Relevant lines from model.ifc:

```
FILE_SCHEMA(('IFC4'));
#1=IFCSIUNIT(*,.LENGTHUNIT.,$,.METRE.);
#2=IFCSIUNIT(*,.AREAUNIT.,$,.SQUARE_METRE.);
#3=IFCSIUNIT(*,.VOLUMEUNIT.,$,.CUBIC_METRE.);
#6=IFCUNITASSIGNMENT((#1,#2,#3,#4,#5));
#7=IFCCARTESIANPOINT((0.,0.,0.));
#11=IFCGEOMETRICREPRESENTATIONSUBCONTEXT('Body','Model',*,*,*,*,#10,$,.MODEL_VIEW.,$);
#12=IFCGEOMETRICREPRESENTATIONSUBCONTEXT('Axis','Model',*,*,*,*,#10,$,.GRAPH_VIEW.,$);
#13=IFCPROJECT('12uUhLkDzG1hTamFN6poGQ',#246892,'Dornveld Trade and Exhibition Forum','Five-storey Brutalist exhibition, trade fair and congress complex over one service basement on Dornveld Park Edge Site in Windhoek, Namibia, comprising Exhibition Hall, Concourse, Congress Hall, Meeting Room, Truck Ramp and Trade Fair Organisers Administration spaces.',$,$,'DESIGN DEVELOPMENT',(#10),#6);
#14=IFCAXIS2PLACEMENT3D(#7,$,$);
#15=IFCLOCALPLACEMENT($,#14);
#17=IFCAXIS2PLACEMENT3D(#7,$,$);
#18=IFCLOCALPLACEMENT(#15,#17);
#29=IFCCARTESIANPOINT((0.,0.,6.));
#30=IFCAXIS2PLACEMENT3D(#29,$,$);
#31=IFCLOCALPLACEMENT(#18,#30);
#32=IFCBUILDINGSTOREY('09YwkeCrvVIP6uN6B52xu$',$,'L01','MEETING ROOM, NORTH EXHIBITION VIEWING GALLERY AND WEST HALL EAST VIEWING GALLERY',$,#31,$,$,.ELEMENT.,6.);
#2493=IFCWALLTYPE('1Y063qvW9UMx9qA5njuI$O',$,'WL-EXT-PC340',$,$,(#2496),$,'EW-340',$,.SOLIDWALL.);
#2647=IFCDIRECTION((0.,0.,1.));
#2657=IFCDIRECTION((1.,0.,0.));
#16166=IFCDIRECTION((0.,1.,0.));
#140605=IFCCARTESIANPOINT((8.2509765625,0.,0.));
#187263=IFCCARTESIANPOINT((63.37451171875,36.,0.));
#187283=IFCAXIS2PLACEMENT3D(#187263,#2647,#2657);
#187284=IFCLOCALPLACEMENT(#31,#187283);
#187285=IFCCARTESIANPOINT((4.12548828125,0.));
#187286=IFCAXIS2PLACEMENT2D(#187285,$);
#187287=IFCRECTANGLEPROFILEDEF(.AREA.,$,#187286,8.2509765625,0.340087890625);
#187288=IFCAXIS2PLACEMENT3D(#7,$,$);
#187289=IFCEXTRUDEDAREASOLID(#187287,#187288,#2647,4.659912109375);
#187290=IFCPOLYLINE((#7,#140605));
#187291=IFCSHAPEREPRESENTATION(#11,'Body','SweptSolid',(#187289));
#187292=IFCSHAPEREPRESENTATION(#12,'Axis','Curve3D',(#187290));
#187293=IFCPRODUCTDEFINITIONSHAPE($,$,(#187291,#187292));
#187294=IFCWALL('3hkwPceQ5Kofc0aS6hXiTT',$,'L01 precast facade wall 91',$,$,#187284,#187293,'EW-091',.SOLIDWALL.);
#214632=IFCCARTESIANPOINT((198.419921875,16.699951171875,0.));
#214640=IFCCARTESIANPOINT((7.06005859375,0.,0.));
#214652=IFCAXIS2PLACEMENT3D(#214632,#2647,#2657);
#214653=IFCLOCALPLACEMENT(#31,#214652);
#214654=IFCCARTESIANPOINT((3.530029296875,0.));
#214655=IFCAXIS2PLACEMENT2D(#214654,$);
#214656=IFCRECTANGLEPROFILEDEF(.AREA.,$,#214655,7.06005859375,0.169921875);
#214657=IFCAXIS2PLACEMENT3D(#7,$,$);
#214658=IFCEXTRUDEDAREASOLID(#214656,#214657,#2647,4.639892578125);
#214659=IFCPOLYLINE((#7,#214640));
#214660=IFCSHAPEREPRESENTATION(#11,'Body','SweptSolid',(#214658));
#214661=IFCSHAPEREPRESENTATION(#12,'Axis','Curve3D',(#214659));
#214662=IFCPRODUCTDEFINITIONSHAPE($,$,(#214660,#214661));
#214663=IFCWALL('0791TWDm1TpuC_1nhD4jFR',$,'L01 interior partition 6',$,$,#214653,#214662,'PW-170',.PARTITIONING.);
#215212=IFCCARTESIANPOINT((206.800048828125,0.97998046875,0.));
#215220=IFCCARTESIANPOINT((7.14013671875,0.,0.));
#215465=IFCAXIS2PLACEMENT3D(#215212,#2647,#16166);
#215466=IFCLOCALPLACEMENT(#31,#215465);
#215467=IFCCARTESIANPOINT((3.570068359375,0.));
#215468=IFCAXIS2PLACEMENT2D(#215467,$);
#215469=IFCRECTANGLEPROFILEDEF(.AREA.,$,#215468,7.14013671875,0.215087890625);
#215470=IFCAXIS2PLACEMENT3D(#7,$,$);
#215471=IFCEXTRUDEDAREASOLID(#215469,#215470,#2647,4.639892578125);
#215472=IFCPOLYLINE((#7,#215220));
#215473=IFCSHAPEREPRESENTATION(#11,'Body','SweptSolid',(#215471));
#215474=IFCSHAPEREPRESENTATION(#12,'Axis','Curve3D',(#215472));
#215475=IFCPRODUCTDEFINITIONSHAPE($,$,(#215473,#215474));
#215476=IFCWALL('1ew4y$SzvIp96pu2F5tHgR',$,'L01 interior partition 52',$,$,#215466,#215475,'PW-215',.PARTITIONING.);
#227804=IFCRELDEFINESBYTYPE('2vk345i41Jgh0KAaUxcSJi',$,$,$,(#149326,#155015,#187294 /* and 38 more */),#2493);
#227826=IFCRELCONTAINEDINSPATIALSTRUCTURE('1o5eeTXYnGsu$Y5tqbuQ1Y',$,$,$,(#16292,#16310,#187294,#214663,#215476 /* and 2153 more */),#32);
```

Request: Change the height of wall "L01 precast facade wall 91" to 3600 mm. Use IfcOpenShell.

```python
import ifcopenshell
import ifcopenshell.geom
import ifcopenshell.util.representation
import ifcopenshell.util.shape
import ifcopenshell.util.unit

model = ifcopenshell.open("model.ifc")
unit_scale = ifcopenshell.util.unit.calculate_unit_scale(model)
settings = ifcopenshell.geom.settings()


def volume(element):
    """Net volume in cubic metres, openings subtracted."""
    shape = ifcopenshell.geom.create_shape(settings, element)
    return ifcopenshell.util.shape.get_volume(shape.geometry)


wall = model.by_guid("3hkwPceQ5Kofc0aS6hXiTT")
before = volume(wall)

body = ifcopenshell.util.representation.get_representation(wall, "Model", "Body")
solid = body.Items[0]
old_height = solid.Depth
solid.Depth = 3.6 / unit_scale
after = volume(wall)

print(f"height {old_height:g} -> {solid.Depth:g}, volume {before:.3f} -> {after:.3f} m3")

model.write("model_v2.ifc")
```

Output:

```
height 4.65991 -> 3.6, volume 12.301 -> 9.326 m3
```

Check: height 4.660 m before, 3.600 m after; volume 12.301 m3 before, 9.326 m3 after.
